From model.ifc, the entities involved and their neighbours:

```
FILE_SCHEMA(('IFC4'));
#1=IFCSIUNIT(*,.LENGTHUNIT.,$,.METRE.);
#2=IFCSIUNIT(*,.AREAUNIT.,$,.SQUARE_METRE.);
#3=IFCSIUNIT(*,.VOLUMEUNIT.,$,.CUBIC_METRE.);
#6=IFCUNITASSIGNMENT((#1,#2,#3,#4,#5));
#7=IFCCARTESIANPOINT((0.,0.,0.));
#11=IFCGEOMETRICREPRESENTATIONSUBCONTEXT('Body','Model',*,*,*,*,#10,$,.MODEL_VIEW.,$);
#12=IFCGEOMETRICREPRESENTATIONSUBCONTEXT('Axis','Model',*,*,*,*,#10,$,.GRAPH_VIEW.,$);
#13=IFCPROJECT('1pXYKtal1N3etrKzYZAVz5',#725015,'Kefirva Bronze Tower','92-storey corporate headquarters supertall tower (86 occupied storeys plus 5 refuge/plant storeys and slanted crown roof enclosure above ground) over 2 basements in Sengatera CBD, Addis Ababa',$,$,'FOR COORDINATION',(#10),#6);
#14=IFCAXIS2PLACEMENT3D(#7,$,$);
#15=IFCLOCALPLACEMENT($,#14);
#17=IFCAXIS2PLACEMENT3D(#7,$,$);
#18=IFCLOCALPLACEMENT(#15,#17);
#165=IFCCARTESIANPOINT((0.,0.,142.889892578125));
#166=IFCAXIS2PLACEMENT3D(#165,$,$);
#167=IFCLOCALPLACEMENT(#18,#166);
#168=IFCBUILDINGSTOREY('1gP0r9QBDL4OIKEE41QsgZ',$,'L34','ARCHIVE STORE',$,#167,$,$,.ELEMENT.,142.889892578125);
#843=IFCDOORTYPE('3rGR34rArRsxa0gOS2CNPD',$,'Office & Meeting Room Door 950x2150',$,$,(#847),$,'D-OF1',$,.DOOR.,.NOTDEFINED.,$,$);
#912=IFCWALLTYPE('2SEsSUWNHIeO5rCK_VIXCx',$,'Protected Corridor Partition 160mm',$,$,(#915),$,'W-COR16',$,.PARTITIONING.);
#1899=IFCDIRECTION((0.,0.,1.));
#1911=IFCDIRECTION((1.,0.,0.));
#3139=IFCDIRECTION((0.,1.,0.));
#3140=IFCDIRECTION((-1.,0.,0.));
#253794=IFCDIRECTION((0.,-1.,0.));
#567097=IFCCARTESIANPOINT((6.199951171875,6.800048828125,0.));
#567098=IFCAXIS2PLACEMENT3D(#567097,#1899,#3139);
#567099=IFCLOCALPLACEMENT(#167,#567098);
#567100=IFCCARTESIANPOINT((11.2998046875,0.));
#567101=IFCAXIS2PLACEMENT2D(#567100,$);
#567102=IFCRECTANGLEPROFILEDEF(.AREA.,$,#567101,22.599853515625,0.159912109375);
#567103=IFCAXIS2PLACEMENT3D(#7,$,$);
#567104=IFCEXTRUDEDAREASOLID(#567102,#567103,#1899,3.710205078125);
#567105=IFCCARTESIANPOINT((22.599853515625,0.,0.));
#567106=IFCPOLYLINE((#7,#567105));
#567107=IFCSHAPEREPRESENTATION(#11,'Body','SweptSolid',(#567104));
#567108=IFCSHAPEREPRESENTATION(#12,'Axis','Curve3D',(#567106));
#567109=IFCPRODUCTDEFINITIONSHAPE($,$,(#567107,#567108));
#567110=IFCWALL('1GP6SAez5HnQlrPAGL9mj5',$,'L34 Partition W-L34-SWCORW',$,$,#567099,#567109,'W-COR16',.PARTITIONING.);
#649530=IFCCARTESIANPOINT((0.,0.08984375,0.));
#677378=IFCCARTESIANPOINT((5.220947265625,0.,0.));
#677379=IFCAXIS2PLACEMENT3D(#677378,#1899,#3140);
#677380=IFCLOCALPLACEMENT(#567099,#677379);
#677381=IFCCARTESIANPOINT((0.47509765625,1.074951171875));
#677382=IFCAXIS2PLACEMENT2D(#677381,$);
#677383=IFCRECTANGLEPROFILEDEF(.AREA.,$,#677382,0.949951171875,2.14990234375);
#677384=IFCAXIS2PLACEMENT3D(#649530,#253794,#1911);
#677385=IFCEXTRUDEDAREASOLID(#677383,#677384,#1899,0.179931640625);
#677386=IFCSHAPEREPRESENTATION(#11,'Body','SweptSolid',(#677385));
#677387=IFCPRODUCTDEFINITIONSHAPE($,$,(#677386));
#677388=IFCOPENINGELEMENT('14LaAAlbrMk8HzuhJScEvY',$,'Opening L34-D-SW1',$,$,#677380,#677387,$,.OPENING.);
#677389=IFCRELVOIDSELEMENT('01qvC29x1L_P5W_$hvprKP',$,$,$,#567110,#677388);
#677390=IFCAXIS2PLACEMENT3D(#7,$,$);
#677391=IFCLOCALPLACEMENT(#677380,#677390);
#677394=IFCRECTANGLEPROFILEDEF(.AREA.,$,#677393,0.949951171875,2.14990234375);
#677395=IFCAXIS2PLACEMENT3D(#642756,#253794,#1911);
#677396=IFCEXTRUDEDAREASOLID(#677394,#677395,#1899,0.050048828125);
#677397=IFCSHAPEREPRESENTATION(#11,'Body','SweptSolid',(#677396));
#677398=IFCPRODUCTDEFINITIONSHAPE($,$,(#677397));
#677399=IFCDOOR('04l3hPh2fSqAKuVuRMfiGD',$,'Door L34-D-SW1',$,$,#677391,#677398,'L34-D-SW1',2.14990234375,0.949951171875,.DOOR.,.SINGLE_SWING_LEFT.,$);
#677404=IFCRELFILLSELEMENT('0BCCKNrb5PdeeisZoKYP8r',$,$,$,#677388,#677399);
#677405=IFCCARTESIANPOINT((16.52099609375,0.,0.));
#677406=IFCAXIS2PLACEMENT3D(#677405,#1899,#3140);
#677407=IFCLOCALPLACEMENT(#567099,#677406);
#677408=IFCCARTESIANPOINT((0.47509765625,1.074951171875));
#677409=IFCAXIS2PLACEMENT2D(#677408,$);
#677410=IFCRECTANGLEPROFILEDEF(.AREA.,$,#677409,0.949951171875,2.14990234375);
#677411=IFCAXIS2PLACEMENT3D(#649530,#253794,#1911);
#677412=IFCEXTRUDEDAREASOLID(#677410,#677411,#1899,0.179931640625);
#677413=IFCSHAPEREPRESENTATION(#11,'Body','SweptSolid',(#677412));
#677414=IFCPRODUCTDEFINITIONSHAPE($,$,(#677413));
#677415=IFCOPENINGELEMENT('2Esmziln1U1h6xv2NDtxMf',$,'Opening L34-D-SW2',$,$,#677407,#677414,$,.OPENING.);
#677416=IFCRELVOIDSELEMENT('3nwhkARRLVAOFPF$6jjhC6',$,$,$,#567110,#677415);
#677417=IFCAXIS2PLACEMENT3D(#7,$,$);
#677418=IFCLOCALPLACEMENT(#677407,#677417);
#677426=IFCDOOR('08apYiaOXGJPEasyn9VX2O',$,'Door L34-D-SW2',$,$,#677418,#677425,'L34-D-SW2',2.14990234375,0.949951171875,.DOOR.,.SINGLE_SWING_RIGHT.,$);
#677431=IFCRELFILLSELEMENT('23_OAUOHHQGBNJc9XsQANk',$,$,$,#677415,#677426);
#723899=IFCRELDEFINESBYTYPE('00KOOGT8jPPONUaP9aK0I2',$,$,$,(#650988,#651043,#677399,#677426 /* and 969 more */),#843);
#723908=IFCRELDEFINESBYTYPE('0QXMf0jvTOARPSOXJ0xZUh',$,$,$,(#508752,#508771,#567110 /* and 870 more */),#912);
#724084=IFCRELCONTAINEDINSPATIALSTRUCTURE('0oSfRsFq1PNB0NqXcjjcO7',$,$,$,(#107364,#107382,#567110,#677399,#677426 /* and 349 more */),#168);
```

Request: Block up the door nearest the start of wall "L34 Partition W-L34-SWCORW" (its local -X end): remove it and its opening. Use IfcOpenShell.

```python
import ifcopenshell
import ifcopenshell.api.feature
import ifcopenshell.api.root
import ifcopenshell.geom
import ifcopenshell.util.shape

model = ifcopenshell.open("model.ifc")
settings = ifcopenshell.geom.settings()


def volume(element):
    """Net volume in cubic metres, openings subtracted."""
    shape = ifcopenshell.geom.create_shape(settings, element)
    return ifcopenshell.util.shape.get_volume(shape.geometry)


door = model.by_guid("04l3hPh2fSqAKuVuRMfiGD")
opening = door.FillsVoids[0].RelatingOpeningElement
wall = opening.VoidsElements[0].RelatingBuildingElement
before = volume(wall)

ifcopenshell.api.root.remove_product(model, product=door)
ifcopenshell.api.feature.remove_feature(model, feature=opening)

after = volume(wall)

print(f"wall volume {before:.3f} -> {after:.3f} m3")

model.write("model-out.ifc")
```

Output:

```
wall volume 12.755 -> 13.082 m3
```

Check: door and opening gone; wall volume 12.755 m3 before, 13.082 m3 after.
